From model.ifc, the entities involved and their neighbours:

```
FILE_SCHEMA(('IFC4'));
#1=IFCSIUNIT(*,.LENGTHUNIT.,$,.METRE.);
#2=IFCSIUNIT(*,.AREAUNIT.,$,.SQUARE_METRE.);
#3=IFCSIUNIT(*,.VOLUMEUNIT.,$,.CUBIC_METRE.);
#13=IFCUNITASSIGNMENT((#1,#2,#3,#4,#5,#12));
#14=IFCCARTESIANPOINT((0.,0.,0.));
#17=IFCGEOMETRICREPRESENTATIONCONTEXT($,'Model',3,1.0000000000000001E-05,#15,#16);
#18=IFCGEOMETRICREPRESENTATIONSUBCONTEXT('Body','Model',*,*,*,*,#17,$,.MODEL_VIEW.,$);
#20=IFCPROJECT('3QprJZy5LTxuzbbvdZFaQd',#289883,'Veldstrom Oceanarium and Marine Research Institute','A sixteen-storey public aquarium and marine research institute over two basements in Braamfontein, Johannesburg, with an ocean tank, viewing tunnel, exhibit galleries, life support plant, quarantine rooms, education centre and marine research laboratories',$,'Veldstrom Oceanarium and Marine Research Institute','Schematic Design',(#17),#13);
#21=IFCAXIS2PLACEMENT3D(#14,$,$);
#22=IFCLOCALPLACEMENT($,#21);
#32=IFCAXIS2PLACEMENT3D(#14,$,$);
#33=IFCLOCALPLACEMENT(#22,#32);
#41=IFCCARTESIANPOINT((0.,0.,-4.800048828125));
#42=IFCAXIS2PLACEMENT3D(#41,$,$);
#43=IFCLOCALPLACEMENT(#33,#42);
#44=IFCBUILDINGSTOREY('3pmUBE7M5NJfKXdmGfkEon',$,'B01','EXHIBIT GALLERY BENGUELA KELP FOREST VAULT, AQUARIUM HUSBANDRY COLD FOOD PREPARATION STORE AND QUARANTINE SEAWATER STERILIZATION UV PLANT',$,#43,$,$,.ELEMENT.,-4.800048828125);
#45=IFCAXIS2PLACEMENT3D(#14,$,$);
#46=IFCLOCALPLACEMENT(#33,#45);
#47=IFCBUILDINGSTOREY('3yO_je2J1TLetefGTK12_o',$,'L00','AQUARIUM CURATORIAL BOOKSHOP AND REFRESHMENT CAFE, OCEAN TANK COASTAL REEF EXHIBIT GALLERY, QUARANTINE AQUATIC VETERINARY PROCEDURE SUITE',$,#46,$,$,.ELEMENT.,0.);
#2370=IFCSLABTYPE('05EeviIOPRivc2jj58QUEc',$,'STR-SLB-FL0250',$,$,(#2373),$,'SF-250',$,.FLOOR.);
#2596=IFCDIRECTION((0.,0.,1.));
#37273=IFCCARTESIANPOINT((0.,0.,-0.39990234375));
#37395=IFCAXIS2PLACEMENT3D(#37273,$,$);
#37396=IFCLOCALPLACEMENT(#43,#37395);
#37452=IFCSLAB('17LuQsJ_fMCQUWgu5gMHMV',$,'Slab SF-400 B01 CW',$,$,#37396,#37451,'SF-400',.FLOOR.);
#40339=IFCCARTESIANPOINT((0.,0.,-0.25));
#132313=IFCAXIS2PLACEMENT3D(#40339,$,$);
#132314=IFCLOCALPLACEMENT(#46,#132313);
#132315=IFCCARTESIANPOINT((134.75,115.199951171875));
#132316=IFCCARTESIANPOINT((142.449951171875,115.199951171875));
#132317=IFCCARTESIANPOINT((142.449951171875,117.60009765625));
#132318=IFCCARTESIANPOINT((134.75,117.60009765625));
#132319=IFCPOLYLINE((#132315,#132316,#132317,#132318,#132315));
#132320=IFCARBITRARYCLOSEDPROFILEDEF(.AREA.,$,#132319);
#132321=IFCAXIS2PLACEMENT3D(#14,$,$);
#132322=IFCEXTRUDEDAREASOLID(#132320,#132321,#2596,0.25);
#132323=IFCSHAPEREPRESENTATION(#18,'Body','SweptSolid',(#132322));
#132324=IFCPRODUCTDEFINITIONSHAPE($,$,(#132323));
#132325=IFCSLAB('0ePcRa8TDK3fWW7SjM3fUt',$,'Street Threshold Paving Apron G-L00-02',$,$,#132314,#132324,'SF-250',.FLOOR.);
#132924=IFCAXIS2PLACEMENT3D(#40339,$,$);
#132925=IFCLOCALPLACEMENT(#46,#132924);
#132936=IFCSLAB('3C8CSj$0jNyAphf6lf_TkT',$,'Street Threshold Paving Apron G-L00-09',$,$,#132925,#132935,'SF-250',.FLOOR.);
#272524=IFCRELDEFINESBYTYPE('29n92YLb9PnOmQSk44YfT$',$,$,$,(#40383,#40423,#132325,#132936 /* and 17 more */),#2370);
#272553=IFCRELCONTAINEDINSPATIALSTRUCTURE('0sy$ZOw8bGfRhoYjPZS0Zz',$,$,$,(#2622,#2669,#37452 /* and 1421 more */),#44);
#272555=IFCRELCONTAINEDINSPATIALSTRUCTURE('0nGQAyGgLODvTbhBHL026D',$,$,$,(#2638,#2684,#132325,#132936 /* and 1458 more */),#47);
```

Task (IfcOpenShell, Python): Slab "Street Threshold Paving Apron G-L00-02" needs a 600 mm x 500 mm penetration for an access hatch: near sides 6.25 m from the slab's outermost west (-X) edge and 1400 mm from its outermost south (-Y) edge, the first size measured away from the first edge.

```python
import numpy as np
import ifcopenshell
import ifcopenshell.api.feature
import ifcopenshell.api.geometry
import ifcopenshell.api.root
import ifcopenshell.geom
import ifcopenshell.util.placement
import ifcopenshell.util.representation
import ifcopenshell.util.shape
import ifcopenshell.util.unit

model = ifcopenshell.open("model.ifc")
unit_scale = ifcopenshell.util.unit.calculate_unit_scale(model)
settings = ifcopenshell.geom.settings()


def volume(element):
    """Net volume in cubic metres, openings subtracted."""
    shape = ifcopenshell.geom.create_shape(settings, element)
    return ifcopenshell.util.shape.get_volume(shape.geometry)


slab = model.by_id(132325)
before = volume(slab)

# Extent in the slab's own axes, in metres. The edges named are its -X and -Y sides.
slab_shape = ifcopenshell.geom.create_shape(settings, slab)
vertices = ifcopenshell.util.shape.get_vertices(slab_shape.geometry)
x_min, y_min, bottom = vertices.min(axis=0)
top = vertices[:, 2].max()

opening = ifcopenshell.api.root.create_entity(model, ifc_class="IfcOpeningElement", name="Access hatch opening", predefined_type="OPENING")
context = ifcopenshell.util.representation.get_context(model, "Model", "Body", "MODEL_VIEW")
width, depth = 0.6, 0.5
outline = [(0.0, 0.0), (width, 0.0), (width, depth), (0.0, depth), (0.0, 0.0)]
# Overshoot both faces by 50 mm so the cut is clean.
shape = ifcopenshell.api.geometry.add_slab_representation(
    model, context=context, depth=top - bottom + 0.1, polyline=outline
)
ifcopenshell.api.geometry.assign_representation(model, product=opening, representation=shape)

matrix = ifcopenshell.util.placement.get_local_placement(slab.ObjectPlacement)
matrix[:, 3] = matrix @ np.append(np.array([x_min + 6.25, y_min + 1.4, bottom - 0.05]) / unit_scale, 1.0)
ifcopenshell.api.geometry.edit_object_placement(model, product=opening, matrix=matrix, is_si=False)
ifcopenshell.api.feature.add_feature(model, feature=opening, element=slab)

after = volume(slab)

print(f"slab volume {before:.3f} -> {after:.3f} m3")

model.write("model_v2.ifc")
```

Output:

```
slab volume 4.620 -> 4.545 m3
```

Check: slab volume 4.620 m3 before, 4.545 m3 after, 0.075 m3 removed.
